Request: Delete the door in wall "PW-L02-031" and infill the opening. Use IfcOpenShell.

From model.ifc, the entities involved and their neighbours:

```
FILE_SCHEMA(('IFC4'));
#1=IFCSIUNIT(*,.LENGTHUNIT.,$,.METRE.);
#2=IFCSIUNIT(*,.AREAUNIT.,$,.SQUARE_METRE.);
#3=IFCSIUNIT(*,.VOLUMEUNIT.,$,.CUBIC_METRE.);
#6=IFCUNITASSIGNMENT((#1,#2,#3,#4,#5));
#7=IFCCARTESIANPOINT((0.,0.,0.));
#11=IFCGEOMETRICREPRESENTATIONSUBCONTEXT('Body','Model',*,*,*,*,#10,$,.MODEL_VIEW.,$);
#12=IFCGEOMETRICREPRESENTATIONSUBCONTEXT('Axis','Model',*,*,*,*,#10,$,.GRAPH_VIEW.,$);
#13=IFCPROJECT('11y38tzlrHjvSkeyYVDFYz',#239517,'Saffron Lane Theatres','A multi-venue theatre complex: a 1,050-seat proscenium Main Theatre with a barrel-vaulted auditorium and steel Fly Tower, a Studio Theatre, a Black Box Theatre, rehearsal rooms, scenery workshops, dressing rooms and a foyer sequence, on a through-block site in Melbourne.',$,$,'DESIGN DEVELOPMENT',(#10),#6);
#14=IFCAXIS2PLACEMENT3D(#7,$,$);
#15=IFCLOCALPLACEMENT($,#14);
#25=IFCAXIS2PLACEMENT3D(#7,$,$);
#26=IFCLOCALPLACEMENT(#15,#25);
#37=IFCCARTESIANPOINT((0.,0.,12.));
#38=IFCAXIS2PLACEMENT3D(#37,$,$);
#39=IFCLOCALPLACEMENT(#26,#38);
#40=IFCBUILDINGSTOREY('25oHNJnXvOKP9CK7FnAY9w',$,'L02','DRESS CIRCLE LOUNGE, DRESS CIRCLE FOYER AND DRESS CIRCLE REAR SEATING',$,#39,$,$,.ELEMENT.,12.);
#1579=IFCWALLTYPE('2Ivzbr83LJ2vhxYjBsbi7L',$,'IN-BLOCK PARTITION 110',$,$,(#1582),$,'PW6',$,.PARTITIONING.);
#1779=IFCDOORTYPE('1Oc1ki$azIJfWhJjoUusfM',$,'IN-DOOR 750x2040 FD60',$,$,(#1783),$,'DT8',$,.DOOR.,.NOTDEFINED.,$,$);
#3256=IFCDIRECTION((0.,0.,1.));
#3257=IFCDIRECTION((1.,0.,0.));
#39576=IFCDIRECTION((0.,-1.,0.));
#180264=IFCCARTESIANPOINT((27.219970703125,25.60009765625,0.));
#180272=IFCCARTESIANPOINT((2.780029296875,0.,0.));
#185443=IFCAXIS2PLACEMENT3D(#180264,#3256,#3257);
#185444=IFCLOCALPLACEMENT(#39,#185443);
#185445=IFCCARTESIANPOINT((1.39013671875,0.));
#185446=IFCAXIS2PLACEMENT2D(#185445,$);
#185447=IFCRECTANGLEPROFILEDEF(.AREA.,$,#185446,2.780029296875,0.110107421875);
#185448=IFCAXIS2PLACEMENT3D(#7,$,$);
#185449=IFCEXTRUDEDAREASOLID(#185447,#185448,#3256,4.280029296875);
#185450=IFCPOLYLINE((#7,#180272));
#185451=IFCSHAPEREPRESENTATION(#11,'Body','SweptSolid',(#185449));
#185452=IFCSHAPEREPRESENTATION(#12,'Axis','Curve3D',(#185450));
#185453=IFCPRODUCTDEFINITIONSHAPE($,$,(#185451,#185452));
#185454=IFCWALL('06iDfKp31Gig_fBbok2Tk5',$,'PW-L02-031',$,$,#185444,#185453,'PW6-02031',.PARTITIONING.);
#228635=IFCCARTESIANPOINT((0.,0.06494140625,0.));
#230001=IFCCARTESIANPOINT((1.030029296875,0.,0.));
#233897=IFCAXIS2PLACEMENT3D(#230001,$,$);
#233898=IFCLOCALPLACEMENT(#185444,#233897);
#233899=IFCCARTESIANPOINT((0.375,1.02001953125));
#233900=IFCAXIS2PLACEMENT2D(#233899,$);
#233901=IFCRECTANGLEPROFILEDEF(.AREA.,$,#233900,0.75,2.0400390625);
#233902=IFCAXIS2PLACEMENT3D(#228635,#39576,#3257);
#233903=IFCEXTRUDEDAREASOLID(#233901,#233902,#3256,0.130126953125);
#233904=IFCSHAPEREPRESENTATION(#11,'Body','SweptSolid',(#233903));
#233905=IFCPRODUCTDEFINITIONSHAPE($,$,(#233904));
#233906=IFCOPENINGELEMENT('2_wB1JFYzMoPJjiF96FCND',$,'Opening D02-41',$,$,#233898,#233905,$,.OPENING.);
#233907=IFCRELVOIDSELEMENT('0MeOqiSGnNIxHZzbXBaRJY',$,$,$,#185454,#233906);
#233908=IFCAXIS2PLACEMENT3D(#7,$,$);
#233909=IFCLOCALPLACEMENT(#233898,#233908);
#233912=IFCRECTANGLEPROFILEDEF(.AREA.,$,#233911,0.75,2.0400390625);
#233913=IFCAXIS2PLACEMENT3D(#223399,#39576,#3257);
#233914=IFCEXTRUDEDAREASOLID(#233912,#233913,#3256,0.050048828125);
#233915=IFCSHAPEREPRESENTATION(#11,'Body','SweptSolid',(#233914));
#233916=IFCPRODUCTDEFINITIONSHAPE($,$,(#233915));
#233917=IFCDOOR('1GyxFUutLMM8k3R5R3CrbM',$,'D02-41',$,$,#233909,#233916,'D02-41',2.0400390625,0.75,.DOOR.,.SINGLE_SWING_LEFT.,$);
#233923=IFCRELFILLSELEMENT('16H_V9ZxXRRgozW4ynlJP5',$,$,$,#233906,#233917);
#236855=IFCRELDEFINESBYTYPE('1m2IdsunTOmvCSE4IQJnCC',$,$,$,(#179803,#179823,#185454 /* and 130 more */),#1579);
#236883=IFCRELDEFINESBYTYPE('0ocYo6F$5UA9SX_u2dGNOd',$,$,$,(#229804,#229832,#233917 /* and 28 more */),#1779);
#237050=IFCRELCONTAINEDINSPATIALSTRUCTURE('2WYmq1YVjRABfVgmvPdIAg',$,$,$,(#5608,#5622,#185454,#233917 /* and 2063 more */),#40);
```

```python
import ifcopenshell
import ifcopenshell.api.feature
import ifcopenshell.api.root
import ifcopenshell.geom
import ifcopenshell.util.shape

model = ifcopenshell.open("model.ifc")
settings = ifcopenshell.geom.settings()


def volume(element):
    """Net volume in cubic metres, openings subtracted."""
    shape = ifcopenshell.geom.create_shape(settings, element)
    return ifcopenshell.util.shape.get_volume(shape.geometry)


door = model.by_id(233917)
opening = door.FillsVoids[0].RelatingOpeningElement
wall = opening.VoidsElements[0].RelatingBuildingElement
before = volume(wall)

ifcopenshell.api.root.remove_product(model, product=door)
ifcopenshell.api.feature.remove_feature(model, feature=opening)

after = volume(wall)

print(f"wall volume {before:.3f} -> {after:.3f} m3")

model.write("model_v2.ifc")
```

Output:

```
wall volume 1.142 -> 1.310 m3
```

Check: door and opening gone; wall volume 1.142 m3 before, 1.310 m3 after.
